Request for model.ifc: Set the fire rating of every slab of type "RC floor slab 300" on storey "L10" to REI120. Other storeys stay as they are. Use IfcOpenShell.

First a look at what the model holds.

```python
import ifcopenshell
import ifcopenshell.util.element

model = ifcopenshell.open("model.ifc")
print(model.schema)
storey = next(s for s in model.by_type("IfcBuildingStorey") if s.Name == "L10")
slabs = [e for e in ifcopenshell.util.element.get_decomposition(storey) if e.is_a("IfcSlab")]
seen = {}
for e in slabs:
    element_type = ifcopenshell.util.element.get_type(e)
    key = (element_type.Name if element_type != e and element_type else None, ifcopenshell.util.element.get_pset(e, "Pset_SlabCommon", "FireRating"))
    seen[key] = seen.get(key, 0) + 1
for (name, value), count in sorted(seen.items(), key=str):
    print(count, "x", name, "|", value)
```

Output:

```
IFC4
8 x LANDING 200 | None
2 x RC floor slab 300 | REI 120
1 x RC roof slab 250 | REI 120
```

```python
import ifcopenshell
import ifcopenshell.api.pset
import ifcopenshell.util.element

model = ifcopenshell.open("model.ifc")

storey = next(s for s in model.by_type("IfcBuildingStorey") if s.Name == "L10")
slabs = [e for e in ifcopenshell.util.element.get_decomposition(storey) if e.is_a("IfcSlab")]

count = 0
for e in slabs:
    element_type = ifcopenshell.util.element.get_type(e)
    if element_type in (None, e) or element_type.Name != "RC floor slab 300":
        continue
    # add_pset returns the element's existing set when there is one.
    pset = ifcopenshell.api.pset.add_pset(model, product=e, name="Pset_SlabCommon")
    ifcopenshell.api.pset.edit_pset(model, pset=pset, properties={"FireRating": "REI120"})
    count += 1

print(count, "slabs updated")

model.write("model_rev.ifc")
```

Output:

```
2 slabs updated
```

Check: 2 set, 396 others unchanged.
